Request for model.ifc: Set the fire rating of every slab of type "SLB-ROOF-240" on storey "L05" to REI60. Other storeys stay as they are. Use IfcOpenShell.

First a look at what the model holds.

```python
import ifcopenshell
import ifcopenshell.util.element

model = ifcopenshell.open("model.ifc")
print(model.schema)
storey = next(s for s in model.by_type("IfcBuildingStorey") if s.Name == "L05")
slabs = [e for e in ifcopenshell.util.element.get_decomposition(storey) if e.is_a("IfcSlab")]
seen = {}
for e in slabs:
    element_type = ifcopenshell.util.element.get_type(e)
    key = (element_type.Name if element_type != e and element_type else None, ifcopenshell.util.element.get_pset(e, "Pset_SlabCommon", "FireRating"))
    seen[key] = seen.get(key, 0) + 1
for (name, value), count in sorted(seen.items(), key=str):
    print(count, "x", name, "|", value)
```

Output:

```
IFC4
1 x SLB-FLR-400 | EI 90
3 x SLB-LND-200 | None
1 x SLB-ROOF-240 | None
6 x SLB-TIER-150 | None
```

```python
import ifcopenshell
import ifcopenshell.api.pset
import ifcopenshell.util.element

model = ifcopenshell.open("model.ifc")

storey = next(s for s in model.by_type("IfcBuildingStorey") if s.Name == "L05")
slabs = [e for e in ifcopenshell.util.element.get_decomposition(storey) if e.is_a("IfcSlab")]

count = 0
for e in slabs:
    element_type = ifcopenshell.util.element.get_type(e)
    if element_type in (None, e) or element_type.Name != "SLB-ROOF-240":
        continue
    # add_pset returns the element's existing set when there is one.
    pset = ifcopenshell.api.pset.add_pset(model, product=e, name="Pset_SlabCommon")
    ifcopenshell.api.pset.edit_pset(model, pset=pset, properties={"FireRating": "REI60"})
    count += 1

print(count, "slabs updated")

model.write("model_v2.ifc")
```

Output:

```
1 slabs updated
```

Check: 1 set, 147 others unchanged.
